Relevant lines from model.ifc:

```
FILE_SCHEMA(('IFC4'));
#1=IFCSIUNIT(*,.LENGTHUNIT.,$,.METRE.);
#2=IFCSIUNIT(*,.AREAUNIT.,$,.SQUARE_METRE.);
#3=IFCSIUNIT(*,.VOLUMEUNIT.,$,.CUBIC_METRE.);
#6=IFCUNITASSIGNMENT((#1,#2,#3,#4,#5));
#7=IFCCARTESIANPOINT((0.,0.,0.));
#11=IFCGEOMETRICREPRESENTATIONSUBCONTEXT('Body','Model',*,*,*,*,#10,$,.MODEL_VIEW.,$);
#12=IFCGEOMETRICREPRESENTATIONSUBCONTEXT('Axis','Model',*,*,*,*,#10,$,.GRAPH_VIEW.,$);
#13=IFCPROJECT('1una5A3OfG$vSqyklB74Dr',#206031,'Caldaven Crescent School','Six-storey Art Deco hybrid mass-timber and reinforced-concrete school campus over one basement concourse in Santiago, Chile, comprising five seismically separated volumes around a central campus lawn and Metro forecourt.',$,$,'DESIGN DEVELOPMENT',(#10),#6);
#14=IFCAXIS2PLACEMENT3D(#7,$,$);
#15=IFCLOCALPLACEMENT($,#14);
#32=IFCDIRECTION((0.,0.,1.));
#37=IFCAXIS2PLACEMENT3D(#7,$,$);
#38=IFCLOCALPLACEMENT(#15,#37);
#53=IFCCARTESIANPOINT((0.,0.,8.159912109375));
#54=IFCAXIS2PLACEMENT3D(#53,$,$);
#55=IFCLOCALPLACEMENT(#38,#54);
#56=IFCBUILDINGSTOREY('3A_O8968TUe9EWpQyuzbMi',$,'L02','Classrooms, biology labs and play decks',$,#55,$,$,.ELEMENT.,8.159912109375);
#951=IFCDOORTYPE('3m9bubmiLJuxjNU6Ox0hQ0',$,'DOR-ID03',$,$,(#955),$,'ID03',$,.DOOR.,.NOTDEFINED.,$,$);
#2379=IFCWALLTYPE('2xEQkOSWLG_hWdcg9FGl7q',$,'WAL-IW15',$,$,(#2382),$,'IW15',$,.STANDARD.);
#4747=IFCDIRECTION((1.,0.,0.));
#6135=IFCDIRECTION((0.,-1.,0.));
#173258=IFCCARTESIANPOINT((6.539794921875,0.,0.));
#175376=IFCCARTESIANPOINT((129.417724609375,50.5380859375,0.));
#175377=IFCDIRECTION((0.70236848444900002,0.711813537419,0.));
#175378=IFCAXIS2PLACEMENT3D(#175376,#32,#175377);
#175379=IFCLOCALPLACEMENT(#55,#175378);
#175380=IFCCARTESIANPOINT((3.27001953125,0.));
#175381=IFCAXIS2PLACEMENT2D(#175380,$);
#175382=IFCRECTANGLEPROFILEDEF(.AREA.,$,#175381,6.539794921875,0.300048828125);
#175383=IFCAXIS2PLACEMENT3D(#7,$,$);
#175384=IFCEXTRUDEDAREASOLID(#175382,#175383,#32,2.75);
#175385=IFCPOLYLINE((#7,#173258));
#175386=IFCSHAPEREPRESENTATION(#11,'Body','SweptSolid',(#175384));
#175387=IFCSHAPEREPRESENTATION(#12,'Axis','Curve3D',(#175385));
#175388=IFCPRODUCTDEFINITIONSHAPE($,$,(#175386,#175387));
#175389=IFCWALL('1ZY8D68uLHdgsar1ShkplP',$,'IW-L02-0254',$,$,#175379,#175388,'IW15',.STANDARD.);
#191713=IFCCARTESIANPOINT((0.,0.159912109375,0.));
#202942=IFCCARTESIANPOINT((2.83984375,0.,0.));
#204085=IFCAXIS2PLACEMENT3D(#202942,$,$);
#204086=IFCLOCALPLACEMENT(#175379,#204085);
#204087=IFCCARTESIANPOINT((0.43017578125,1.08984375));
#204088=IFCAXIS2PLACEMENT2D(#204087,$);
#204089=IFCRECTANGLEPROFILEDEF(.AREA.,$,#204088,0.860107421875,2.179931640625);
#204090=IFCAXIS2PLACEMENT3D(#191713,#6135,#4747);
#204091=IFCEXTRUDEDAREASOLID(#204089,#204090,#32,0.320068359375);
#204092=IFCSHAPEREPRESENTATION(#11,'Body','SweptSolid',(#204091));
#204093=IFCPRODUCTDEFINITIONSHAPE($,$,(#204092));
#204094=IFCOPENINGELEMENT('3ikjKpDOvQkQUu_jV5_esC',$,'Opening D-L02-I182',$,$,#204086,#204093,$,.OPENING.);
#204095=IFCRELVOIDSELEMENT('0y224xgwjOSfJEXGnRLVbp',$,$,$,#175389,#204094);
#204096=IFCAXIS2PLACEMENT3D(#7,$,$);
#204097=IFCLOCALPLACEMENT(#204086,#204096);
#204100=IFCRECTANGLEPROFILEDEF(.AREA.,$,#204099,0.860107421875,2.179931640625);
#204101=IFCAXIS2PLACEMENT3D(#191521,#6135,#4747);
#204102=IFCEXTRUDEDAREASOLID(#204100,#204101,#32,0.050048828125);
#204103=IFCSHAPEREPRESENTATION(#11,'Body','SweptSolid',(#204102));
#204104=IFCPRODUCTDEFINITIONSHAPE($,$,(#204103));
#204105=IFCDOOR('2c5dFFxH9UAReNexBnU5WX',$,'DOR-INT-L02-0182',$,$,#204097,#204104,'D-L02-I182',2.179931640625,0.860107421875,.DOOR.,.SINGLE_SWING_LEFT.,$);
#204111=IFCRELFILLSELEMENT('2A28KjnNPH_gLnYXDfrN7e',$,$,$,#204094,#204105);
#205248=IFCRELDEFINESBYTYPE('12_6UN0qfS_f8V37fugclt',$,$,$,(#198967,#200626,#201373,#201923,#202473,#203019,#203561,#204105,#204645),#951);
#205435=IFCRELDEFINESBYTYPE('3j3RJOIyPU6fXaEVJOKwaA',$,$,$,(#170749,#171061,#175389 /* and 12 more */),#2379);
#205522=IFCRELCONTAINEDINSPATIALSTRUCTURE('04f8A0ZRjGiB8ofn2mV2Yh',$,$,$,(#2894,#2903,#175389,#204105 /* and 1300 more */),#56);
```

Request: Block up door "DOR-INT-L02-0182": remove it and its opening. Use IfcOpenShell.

```python
import ifcopenshell
import ifcopenshell.api.feature
import ifcopenshell.api.root
import ifcopenshell.geom
import ifcopenshell.util.shape

model = ifcopenshell.open("model.ifc")
settings = ifcopenshell.geom.settings()


def volume(element):
    """Net volume in cubic metres, openings subtracted."""
    shape = ifcopenshell.geom.create_shape(settings, element)
    return ifcopenshell.util.shape.get_volume(shape.geometry)


door = model.by_guid("2c5dFFxH9UAReNexBnU5WX")
opening = door.FillsVoids[0].RelatingOpeningElement
wall = opening.VoidsElements[0].RelatingBuildingElement
before = volume(wall)

ifcopenshell.api.root.remove_product(model, product=door)
ifcopenshell.api.feature.remove_feature(model, feature=opening)

after = volume(wall)

print(f"wall volume {before:.3f} -> {after:.3f} m3")

model.write("model_updated.ifc")
```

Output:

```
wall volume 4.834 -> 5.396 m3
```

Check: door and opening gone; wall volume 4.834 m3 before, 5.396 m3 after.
